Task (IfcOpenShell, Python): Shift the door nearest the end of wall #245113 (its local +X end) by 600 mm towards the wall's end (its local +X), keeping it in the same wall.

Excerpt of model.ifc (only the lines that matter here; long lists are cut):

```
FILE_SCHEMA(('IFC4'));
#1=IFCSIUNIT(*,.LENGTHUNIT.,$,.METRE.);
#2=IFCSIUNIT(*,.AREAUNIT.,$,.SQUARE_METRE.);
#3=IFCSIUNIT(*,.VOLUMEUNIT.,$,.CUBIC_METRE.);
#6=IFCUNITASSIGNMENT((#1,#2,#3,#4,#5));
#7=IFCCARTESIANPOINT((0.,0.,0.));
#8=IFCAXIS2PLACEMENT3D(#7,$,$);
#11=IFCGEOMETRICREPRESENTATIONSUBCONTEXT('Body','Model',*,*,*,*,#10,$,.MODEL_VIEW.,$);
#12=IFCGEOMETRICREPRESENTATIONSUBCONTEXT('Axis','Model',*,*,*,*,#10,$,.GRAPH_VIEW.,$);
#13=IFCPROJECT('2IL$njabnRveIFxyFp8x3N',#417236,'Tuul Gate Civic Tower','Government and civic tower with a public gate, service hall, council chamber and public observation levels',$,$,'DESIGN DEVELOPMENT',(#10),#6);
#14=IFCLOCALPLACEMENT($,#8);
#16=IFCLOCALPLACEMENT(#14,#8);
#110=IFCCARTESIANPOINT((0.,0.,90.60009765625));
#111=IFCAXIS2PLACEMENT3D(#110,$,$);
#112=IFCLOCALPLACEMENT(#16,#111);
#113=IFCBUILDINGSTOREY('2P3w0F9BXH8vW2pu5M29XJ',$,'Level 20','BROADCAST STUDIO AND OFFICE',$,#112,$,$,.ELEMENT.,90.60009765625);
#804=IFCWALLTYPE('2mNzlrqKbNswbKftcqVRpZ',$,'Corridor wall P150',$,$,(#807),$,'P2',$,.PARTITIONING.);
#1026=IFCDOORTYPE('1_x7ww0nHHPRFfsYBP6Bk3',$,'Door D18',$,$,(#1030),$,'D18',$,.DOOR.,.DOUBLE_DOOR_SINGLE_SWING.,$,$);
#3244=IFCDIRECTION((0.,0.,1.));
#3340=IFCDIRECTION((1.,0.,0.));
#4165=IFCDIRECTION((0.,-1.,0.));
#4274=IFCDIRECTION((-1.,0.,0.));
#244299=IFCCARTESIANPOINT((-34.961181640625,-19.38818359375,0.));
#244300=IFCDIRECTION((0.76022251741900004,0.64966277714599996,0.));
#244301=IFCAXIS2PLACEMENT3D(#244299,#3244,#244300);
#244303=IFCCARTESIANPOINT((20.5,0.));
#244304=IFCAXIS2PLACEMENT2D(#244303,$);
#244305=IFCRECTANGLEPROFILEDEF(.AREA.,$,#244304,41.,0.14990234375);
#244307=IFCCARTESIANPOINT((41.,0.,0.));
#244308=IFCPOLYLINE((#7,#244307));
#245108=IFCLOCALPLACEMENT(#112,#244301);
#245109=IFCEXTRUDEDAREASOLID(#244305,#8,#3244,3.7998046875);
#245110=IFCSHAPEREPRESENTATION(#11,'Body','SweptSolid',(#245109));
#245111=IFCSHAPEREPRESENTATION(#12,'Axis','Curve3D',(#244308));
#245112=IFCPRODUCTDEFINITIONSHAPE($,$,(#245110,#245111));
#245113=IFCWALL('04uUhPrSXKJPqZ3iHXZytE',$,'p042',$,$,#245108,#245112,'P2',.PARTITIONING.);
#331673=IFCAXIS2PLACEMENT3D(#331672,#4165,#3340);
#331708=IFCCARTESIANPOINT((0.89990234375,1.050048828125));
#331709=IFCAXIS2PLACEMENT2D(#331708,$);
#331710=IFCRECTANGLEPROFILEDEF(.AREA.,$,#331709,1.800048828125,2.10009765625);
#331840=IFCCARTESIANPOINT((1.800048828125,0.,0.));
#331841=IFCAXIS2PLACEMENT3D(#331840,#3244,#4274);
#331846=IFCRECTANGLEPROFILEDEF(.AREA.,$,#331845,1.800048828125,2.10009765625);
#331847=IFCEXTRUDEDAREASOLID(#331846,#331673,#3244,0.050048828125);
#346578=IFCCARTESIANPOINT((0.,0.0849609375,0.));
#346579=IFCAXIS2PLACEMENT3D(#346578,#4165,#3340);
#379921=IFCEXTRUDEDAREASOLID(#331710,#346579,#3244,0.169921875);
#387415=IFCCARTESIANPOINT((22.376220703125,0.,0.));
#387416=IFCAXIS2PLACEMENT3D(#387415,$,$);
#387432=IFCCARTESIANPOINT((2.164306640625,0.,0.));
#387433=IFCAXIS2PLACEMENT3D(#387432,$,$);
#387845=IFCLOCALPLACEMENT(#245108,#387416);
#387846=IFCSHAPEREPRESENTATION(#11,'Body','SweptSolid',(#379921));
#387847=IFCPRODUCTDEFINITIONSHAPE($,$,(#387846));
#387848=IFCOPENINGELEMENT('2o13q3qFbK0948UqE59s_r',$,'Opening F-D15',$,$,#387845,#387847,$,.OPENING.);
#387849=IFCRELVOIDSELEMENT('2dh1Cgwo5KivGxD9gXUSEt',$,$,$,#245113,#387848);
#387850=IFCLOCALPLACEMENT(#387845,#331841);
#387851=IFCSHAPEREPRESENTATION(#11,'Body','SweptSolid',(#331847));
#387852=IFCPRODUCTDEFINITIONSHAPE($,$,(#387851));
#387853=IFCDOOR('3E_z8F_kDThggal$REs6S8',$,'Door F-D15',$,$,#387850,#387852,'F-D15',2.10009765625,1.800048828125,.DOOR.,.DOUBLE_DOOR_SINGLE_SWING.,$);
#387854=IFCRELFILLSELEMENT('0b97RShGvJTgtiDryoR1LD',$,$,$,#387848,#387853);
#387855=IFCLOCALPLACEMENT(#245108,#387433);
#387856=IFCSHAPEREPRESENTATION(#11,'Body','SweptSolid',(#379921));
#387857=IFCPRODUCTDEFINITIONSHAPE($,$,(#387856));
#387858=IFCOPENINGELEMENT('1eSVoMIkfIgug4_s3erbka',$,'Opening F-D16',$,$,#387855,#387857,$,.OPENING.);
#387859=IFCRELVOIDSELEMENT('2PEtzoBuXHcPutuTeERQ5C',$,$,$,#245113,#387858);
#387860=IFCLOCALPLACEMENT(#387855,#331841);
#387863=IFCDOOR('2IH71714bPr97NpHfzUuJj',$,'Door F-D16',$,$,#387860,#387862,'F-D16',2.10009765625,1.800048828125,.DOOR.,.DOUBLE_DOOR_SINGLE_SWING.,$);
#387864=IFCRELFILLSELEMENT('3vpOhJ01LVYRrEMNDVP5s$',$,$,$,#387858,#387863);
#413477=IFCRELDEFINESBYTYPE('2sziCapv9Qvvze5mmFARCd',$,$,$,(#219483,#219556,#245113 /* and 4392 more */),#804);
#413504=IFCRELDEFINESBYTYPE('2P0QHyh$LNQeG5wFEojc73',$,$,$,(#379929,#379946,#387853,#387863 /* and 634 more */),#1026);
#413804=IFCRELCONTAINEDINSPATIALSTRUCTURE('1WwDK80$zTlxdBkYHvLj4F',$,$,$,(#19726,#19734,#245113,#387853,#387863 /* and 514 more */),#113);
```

```python
import ifcopenshell
import ifcopenshell.api.geometry
import ifcopenshell.util.placement
import ifcopenshell.util.unit

model = ifcopenshell.open("model.ifc")
unit_scale = ifcopenshell.util.unit.calculate_unit_scale(model)

door = model.by_guid("3E_z8F_kDThggal$REs6S8")
opening = door.FillsVoids[0].RelatingOpeningElement
wall = opening.VoidsElements[0].RelatingBuildingElement

wall_matrix = ifcopenshell.util.placement.get_local_placement(wall.ObjectPlacement)
shift = wall_matrix[:3, 0] * 0.6 / unit_scale
before = ifcopenshell.util.placement.get_local_placement(door.ObjectPlacement)[:3, 3].copy()

# The door is placed relative to its opening, so it follows when the opening moves.
matrix = ifcopenshell.util.placement.get_local_placement(opening.ObjectPlacement)
matrix[:3, 3] += shift
ifcopenshell.api.geometry.edit_object_placement(
    model, product=opening, matrix=matrix, is_si=False, should_transform_children=True
)

after = ifcopenshell.util.placement.get_local_placement(door.ObjectPlacement)[:3, 3]
print("door moved by", (after - before).round(3) + 0.0)

model.write("model_v2.ifc")
```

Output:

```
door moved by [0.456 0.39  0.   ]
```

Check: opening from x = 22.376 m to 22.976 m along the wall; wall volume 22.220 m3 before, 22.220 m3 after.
